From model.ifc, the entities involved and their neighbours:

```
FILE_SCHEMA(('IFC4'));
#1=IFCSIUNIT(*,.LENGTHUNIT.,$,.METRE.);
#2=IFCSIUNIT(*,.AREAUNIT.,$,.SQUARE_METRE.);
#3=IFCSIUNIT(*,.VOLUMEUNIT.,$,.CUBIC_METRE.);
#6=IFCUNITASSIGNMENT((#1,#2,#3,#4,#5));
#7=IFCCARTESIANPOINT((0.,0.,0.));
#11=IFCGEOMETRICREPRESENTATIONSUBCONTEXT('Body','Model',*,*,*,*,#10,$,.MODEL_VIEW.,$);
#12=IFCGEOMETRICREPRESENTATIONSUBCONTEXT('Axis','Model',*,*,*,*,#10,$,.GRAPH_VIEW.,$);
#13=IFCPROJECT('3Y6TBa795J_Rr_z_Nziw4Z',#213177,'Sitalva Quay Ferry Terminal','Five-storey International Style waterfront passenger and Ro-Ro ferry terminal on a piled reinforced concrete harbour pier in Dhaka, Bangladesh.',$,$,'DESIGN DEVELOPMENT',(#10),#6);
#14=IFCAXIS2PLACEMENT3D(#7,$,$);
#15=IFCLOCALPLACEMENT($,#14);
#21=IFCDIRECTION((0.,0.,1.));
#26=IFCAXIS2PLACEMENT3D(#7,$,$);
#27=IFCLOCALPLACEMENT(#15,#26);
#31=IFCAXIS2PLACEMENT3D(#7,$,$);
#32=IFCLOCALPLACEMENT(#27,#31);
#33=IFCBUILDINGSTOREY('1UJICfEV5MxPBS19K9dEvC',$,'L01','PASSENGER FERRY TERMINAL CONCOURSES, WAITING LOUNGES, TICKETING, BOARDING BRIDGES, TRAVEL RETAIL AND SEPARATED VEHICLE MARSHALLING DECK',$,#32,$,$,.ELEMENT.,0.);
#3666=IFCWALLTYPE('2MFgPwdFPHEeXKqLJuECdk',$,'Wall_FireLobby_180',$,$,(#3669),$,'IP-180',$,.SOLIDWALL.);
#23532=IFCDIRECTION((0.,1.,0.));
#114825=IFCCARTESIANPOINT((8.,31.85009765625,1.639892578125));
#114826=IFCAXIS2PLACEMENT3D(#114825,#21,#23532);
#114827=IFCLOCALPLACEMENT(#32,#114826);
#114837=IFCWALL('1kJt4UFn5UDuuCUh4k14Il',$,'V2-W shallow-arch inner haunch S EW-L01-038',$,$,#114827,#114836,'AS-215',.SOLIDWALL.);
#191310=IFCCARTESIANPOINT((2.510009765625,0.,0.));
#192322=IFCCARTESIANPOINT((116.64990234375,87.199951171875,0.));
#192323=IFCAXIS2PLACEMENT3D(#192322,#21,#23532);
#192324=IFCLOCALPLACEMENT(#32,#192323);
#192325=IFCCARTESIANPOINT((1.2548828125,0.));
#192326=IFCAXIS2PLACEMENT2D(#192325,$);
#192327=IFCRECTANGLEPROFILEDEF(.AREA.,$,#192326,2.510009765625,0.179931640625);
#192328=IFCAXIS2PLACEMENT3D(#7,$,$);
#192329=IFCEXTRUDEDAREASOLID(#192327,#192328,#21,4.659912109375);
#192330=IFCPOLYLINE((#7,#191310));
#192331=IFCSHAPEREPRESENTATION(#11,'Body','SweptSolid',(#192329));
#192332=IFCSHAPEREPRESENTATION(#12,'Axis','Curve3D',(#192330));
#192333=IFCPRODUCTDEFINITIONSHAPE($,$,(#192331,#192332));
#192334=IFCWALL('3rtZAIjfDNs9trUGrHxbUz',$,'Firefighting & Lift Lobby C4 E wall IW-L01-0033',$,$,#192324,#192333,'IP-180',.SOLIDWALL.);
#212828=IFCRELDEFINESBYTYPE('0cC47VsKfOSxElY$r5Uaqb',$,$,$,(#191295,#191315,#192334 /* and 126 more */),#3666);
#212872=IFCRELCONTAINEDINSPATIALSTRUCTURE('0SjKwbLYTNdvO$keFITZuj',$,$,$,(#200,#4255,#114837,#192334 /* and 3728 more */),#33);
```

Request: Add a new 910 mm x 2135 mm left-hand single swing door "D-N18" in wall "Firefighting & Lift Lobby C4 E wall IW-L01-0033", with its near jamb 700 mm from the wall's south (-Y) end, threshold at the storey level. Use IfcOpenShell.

```python
import numpy as np
import ifcopenshell
import ifcopenshell.api.feature
import ifcopenshell.api.geometry
import ifcopenshell.api.root
import ifcopenshell.api.spatial
import ifcopenshell.geom
import ifcopenshell.util.element
import ifcopenshell.util.placement
import ifcopenshell.util.representation
import ifcopenshell.util.shape
import ifcopenshell.util.unit

model = ifcopenshell.open("model.ifc")
unit_scale = ifcopenshell.util.unit.calculate_unit_scale(model)
settings = ifcopenshell.geom.settings()


def volume(element):
    """Net volume in cubic metres, openings subtracted."""
    shape = ifcopenshell.geom.create_shape(settings, element)
    return ifcopenshell.util.shape.get_volume(shape.geometry)


wall = model.by_guid("3rtZAIjfDNs9trUGrHxbUz")
storey = ifcopenshell.util.element.get_container(wall, ifc_class="IfcBuildingStorey")
context = ifcopenshell.util.representation.get_context(model, "Model", "Body", "MODEL_VIEW")
before = volume(wall)

width, height, from_end, sill = 0.91, 2.135, 0.7, 0.0  # metres

# The wall runs along its own X axis, and the end named is its -X end.
wall_shape = ifcopenshell.geom.create_shape(settings, wall)
x, y, z = ifcopenshell.util.shape.get_vertices(wall_shape.geometry).T
start = x.min() + from_end
face, thickness = float(y.min()), float(y.max() - y.min())
wall_matrix = ifcopenshell.util.placement.get_local_placement(wall.ObjectPlacement)
level = ifcopenshell.util.placement.get_local_placement(storey.ObjectPlacement)[2, 3]


def in_wall(x, y):
    """Placement at x, y metres in the wall's axes, at sill height."""
    matrix = wall_matrix.copy()
    matrix[:, 3] = wall_matrix @ np.array([x / unit_scale, y / unit_scale, 0.0, 1.0])
    matrix[2, 3] = level + sill / unit_scale
    return matrix


# Opening: a box that overshoots both wall faces by 50 mm.
opening = ifcopenshell.api.root.create_entity(model, ifc_class="IfcOpeningElement", predefined_type="OPENING")
box = ifcopenshell.api.geometry.add_wall_representation(
    model, context=context, length=width, height=height, thickness=thickness + 0.1
)
ifcopenshell.api.geometry.assign_representation(model, product=opening, representation=box)
ifcopenshell.api.geometry.edit_object_placement(model, product=opening, matrix=in_wall(start, face - 0.05), is_si=False)
ifcopenshell.api.feature.add_feature(model, feature=opening, element=wall)

door = ifcopenshell.api.root.create_entity(model, ifc_class="IfcDoor", name="D-N18", predefined_type="DOOR")
door.OverallWidth, door.OverallHeight = width / unit_scale, height / unit_scale
door.OperationType = "SINGLE_SWING_LEFT"
body = ifcopenshell.api.geometry.add_door_representation(
    model,
    context=context,
    overall_width=door.OverallWidth,
    overall_height=door.OverallHeight,
    operation_type="SINGLE_SWING_LEFT",
    lining_properties={"LiningDepth": thickness / unit_scale, "ThresholdDepth": thickness / unit_scale},
)
ifcopenshell.api.geometry.assign_representation(model, product=door, representation=body)
ifcopenshell.api.spatial.assign_container(model, products=[door], relating_structure=storey)
ifcopenshell.api.feature.add_filling(model, opening=opening, element=door)

# The lining spans the wall, so the door starts at the wall face.
ifcopenshell.api.geometry.edit_object_placement(model, product=door, matrix=in_wall(start, face), is_si=False)

after = volume(wall)

print(f"wall volume {before:.3f} -> {after:.3f} m3")

model.write("model_v2.ifc")
```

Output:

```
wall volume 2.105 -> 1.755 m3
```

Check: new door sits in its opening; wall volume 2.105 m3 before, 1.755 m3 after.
